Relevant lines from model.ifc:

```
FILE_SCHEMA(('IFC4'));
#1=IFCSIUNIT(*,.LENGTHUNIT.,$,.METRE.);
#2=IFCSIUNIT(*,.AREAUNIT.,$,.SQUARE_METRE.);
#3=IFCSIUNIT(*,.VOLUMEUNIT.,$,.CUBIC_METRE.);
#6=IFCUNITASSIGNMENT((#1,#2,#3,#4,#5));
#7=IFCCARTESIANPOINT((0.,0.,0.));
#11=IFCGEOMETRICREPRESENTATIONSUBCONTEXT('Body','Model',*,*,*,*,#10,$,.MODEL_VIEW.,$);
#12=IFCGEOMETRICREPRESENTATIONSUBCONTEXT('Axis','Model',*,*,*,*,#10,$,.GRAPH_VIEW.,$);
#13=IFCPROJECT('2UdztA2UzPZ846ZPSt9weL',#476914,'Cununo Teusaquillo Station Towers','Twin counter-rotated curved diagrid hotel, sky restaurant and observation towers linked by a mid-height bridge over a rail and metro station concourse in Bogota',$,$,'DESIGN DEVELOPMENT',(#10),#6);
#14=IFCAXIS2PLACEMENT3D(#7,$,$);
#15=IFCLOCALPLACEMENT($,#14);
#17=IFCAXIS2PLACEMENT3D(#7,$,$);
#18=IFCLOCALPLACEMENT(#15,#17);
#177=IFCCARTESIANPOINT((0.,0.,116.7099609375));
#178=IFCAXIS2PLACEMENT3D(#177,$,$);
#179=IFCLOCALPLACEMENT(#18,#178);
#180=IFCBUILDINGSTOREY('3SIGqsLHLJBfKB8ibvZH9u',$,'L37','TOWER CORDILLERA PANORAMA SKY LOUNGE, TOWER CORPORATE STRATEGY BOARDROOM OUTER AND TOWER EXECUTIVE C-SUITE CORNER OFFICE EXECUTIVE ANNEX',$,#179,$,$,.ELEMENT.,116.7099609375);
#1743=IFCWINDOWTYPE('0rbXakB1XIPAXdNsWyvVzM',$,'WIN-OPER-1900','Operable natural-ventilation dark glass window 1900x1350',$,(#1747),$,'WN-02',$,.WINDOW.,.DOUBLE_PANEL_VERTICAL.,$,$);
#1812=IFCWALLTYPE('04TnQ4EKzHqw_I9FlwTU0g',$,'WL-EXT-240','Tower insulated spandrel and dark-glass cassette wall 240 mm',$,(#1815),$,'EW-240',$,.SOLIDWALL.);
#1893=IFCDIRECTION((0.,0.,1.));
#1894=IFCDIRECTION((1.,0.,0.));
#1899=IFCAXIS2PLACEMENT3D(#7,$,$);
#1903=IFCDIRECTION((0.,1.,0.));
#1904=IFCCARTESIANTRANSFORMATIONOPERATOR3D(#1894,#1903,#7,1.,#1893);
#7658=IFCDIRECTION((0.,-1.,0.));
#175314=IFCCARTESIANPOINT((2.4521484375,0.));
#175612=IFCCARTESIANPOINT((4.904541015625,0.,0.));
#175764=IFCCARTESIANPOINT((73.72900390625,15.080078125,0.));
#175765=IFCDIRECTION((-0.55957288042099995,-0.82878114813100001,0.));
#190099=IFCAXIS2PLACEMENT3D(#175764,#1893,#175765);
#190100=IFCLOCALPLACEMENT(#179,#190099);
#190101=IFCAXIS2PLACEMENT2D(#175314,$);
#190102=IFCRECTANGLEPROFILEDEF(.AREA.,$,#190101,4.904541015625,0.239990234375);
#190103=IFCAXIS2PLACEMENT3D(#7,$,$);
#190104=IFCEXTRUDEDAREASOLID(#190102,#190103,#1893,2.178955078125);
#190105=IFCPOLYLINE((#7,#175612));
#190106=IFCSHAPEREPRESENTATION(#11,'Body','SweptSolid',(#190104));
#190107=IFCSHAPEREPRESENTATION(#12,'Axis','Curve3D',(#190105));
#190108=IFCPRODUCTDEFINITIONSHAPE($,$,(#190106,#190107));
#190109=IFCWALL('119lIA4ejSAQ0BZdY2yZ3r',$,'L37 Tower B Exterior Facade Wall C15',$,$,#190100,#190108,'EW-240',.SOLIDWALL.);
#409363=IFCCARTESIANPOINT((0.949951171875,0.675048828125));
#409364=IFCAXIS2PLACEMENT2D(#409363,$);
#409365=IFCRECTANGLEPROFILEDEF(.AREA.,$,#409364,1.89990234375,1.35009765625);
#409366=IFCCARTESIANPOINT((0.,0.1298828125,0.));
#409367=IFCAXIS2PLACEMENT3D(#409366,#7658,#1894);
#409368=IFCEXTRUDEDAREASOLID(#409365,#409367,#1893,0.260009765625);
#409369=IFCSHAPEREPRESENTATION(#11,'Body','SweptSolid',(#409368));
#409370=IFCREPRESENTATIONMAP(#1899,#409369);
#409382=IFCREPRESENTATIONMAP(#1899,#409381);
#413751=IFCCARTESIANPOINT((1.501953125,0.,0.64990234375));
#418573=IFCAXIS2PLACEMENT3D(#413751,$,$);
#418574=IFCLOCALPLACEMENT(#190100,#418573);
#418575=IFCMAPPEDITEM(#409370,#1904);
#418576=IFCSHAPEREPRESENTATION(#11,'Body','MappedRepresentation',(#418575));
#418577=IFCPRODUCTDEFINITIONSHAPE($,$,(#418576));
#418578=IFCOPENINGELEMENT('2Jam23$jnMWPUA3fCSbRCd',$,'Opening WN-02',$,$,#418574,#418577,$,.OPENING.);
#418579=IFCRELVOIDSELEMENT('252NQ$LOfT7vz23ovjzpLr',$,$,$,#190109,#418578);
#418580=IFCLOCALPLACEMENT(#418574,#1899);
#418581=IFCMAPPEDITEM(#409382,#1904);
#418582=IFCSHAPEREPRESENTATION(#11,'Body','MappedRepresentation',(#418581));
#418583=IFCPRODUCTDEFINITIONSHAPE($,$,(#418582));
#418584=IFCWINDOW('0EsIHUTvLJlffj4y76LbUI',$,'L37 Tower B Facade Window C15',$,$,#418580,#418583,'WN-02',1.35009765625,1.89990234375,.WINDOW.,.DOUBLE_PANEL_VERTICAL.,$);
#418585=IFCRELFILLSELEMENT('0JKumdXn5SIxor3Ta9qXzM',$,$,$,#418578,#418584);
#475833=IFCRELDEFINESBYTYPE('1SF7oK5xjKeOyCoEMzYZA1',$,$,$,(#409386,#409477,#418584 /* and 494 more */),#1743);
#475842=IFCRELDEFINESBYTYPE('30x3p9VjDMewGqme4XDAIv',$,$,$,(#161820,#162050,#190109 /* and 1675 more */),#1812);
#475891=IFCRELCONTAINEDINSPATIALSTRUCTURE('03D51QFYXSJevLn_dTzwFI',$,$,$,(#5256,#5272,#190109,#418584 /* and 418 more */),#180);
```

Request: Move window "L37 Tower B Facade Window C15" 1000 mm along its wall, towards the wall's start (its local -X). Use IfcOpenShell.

```python
import ifcopenshell
import ifcopenshell.api.geometry
import ifcopenshell.util.placement
import ifcopenshell.util.unit

model = ifcopenshell.open("model.ifc")
unit_scale = ifcopenshell.util.unit.calculate_unit_scale(model)

window = model.by_guid("0EsIHUTvLJlffj4y76LbUI")
opening = window.FillsVoids[0].RelatingOpeningElement
wall = opening.VoidsElements[0].RelatingBuildingElement

wall_matrix = ifcopenshell.util.placement.get_local_placement(wall.ObjectPlacement)
shift = wall_matrix[:3, 0] * -1 / unit_scale
before = ifcopenshell.util.placement.get_local_placement(window.ObjectPlacement)[:3, 3].copy()

# The window is placed relative to its opening, so it follows when the opening moves.
matrix = ifcopenshell.util.placement.get_local_placement(opening.ObjectPlacement)
matrix[:3, 3] += shift
ifcopenshell.api.geometry.edit_object_placement(
    model, product=opening, matrix=matrix, is_si=False, should_transform_children=True
)

after = ifcopenshell.util.placement.get_local_placement(window.ObjectPlacement)[:3, 3]
print("window moved by", (after - before).round(3) + 0.0)

model.write("model_v2.ifc")
```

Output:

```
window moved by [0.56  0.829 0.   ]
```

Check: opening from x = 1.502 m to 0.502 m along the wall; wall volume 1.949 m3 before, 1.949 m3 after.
